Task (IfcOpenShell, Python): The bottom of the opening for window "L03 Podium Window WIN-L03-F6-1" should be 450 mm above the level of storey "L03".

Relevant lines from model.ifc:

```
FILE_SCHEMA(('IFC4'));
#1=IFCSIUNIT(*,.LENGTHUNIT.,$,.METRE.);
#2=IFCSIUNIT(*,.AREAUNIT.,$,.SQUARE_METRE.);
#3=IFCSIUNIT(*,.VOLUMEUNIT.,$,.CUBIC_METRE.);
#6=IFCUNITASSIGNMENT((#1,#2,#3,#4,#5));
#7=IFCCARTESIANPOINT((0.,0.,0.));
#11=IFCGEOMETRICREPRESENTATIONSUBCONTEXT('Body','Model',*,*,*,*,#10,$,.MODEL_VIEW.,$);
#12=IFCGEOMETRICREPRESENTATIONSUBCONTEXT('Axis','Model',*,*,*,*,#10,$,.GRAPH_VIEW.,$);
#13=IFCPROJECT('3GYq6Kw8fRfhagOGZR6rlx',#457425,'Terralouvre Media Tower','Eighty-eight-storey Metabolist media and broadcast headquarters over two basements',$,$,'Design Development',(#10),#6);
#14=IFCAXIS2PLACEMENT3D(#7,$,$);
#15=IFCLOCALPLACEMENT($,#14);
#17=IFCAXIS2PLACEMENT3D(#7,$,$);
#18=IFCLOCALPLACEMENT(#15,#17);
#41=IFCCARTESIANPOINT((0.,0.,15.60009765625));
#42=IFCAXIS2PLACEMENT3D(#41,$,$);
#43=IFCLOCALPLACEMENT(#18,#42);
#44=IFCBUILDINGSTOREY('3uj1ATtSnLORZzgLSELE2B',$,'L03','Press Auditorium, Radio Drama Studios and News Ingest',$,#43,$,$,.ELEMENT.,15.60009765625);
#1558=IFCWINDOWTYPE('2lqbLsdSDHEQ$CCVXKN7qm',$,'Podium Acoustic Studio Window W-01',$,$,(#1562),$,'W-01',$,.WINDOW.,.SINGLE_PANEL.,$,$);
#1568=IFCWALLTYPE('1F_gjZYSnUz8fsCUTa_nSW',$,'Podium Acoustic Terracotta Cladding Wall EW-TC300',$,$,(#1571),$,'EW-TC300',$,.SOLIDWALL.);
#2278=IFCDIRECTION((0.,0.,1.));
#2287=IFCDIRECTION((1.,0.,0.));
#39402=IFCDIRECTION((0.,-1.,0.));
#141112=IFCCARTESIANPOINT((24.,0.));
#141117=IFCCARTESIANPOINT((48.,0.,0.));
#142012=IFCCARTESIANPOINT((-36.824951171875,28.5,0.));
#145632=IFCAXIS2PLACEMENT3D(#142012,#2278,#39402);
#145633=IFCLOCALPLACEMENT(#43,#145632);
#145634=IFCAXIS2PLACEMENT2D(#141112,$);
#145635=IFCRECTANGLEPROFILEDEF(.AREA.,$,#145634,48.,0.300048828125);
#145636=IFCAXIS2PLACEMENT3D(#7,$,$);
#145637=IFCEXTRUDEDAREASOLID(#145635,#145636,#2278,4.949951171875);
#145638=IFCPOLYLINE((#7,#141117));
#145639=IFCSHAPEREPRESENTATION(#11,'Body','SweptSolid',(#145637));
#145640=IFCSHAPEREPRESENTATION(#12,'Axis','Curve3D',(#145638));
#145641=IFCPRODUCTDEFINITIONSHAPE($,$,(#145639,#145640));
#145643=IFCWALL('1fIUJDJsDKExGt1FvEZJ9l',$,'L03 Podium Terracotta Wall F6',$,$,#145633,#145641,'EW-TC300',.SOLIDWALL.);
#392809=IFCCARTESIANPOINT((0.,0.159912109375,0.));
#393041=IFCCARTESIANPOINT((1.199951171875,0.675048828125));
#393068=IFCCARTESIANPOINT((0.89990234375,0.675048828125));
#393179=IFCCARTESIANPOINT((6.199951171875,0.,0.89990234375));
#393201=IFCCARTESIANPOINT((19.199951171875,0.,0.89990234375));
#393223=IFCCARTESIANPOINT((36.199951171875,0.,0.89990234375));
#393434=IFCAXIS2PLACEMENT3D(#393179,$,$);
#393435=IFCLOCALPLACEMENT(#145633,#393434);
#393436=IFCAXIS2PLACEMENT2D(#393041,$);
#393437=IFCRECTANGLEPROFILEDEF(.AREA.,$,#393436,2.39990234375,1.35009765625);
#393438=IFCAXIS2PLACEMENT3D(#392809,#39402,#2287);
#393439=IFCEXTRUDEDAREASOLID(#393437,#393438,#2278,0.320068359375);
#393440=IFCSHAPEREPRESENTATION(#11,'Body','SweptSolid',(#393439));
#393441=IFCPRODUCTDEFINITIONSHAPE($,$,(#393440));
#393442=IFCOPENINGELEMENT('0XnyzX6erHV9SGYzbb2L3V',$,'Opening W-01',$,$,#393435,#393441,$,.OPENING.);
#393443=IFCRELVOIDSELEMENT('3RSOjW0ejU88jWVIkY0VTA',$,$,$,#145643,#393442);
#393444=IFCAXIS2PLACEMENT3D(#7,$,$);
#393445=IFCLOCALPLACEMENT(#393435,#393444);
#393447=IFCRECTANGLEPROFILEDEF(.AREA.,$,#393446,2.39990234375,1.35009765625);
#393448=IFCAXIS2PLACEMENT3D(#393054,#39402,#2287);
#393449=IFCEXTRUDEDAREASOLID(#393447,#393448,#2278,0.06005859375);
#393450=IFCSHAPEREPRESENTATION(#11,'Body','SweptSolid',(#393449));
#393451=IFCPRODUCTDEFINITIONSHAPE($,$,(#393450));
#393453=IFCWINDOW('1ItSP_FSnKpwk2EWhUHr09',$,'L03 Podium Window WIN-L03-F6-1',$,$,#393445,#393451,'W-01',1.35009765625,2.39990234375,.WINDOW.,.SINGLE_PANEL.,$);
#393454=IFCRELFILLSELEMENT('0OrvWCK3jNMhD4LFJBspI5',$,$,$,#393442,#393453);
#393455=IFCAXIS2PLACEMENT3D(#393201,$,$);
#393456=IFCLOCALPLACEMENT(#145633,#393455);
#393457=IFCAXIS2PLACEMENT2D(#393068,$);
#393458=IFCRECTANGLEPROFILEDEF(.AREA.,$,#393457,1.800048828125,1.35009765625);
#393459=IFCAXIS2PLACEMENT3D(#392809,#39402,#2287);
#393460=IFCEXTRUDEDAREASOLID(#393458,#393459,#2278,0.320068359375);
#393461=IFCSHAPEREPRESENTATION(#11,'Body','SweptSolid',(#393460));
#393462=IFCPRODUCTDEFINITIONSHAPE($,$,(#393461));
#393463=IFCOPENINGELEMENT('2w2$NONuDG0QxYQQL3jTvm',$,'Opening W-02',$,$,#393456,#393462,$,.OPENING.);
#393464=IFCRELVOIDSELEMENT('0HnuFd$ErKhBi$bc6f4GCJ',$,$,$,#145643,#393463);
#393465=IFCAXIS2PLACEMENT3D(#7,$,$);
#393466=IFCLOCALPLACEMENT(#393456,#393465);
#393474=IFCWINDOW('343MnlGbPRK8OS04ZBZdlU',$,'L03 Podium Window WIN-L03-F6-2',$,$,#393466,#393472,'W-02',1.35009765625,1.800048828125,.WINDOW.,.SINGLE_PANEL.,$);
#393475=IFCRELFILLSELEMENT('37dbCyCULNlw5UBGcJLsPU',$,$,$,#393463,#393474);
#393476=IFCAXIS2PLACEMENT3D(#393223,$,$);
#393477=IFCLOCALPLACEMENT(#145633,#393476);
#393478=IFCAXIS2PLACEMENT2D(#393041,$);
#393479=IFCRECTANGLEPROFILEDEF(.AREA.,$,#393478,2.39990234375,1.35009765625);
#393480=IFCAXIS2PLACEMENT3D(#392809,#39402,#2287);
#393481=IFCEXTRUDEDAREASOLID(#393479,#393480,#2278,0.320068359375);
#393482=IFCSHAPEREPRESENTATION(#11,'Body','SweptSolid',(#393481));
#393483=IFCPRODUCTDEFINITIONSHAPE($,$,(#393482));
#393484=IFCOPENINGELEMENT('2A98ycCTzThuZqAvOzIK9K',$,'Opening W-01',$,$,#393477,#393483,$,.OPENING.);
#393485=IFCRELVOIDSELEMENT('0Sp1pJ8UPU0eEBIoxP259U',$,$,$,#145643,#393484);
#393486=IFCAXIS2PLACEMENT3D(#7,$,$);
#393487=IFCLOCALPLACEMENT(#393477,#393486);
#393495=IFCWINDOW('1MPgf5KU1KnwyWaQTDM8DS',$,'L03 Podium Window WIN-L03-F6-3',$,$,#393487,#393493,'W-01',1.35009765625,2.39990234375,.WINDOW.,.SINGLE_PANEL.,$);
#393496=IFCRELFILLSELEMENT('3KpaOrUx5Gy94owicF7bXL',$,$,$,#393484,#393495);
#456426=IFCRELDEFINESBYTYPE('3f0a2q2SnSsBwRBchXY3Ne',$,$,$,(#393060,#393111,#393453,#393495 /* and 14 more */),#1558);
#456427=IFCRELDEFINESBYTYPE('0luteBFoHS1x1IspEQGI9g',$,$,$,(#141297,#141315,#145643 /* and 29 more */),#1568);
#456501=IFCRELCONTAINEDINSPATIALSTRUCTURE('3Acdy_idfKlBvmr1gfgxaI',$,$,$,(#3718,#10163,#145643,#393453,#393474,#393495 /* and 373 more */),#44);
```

```python
import numpy as np
import ifcopenshell
import ifcopenshell.api.geometry
import ifcopenshell.geom
import ifcopenshell.util.element
import ifcopenshell.util.placement
import ifcopenshell.util.shape
import ifcopenshell.util.unit

model = ifcopenshell.open("model.ifc")
unit_scale = ifcopenshell.util.unit.calculate_unit_scale(model)

window = model.by_guid("1ItSP_FSnKpwk2EWhUHr09")
opening = window.FillsVoids[0].RelatingOpeningElement
storey = ifcopenshell.util.element.get_container(window, ifc_class="IfcBuildingStorey")
level = ifcopenshell.util.placement.get_local_placement(storey.ObjectPlacement)[2, 3]

# The opening's origin need not be at the sill, so measure its lowest point.
shape = ifcopenshell.geom.create_shape(ifcopenshell.geom.settings(), opening)
bottom = ifcopenshell.util.shape.get_shape_bottom_elevation(shape, shape.geometry) / unit_scale
dz = level + 0.45 / unit_scale - bottom

shift = np.array([0.0, 0.0, dz])
# The window is placed relative to its opening, so it follows when the opening moves.
matrix = ifcopenshell.util.placement.get_local_placement(opening.ObjectPlacement)
matrix[:3, 3] += shift
ifcopenshell.api.geometry.edit_object_placement(
    model, product=opening, matrix=matrix, is_si=False, should_transform_children=True
)

print(f"moved by {dz * unit_scale:+.3f} m")

model.write("model_rev.ifc")
```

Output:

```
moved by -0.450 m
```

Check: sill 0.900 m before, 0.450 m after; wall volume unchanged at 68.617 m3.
